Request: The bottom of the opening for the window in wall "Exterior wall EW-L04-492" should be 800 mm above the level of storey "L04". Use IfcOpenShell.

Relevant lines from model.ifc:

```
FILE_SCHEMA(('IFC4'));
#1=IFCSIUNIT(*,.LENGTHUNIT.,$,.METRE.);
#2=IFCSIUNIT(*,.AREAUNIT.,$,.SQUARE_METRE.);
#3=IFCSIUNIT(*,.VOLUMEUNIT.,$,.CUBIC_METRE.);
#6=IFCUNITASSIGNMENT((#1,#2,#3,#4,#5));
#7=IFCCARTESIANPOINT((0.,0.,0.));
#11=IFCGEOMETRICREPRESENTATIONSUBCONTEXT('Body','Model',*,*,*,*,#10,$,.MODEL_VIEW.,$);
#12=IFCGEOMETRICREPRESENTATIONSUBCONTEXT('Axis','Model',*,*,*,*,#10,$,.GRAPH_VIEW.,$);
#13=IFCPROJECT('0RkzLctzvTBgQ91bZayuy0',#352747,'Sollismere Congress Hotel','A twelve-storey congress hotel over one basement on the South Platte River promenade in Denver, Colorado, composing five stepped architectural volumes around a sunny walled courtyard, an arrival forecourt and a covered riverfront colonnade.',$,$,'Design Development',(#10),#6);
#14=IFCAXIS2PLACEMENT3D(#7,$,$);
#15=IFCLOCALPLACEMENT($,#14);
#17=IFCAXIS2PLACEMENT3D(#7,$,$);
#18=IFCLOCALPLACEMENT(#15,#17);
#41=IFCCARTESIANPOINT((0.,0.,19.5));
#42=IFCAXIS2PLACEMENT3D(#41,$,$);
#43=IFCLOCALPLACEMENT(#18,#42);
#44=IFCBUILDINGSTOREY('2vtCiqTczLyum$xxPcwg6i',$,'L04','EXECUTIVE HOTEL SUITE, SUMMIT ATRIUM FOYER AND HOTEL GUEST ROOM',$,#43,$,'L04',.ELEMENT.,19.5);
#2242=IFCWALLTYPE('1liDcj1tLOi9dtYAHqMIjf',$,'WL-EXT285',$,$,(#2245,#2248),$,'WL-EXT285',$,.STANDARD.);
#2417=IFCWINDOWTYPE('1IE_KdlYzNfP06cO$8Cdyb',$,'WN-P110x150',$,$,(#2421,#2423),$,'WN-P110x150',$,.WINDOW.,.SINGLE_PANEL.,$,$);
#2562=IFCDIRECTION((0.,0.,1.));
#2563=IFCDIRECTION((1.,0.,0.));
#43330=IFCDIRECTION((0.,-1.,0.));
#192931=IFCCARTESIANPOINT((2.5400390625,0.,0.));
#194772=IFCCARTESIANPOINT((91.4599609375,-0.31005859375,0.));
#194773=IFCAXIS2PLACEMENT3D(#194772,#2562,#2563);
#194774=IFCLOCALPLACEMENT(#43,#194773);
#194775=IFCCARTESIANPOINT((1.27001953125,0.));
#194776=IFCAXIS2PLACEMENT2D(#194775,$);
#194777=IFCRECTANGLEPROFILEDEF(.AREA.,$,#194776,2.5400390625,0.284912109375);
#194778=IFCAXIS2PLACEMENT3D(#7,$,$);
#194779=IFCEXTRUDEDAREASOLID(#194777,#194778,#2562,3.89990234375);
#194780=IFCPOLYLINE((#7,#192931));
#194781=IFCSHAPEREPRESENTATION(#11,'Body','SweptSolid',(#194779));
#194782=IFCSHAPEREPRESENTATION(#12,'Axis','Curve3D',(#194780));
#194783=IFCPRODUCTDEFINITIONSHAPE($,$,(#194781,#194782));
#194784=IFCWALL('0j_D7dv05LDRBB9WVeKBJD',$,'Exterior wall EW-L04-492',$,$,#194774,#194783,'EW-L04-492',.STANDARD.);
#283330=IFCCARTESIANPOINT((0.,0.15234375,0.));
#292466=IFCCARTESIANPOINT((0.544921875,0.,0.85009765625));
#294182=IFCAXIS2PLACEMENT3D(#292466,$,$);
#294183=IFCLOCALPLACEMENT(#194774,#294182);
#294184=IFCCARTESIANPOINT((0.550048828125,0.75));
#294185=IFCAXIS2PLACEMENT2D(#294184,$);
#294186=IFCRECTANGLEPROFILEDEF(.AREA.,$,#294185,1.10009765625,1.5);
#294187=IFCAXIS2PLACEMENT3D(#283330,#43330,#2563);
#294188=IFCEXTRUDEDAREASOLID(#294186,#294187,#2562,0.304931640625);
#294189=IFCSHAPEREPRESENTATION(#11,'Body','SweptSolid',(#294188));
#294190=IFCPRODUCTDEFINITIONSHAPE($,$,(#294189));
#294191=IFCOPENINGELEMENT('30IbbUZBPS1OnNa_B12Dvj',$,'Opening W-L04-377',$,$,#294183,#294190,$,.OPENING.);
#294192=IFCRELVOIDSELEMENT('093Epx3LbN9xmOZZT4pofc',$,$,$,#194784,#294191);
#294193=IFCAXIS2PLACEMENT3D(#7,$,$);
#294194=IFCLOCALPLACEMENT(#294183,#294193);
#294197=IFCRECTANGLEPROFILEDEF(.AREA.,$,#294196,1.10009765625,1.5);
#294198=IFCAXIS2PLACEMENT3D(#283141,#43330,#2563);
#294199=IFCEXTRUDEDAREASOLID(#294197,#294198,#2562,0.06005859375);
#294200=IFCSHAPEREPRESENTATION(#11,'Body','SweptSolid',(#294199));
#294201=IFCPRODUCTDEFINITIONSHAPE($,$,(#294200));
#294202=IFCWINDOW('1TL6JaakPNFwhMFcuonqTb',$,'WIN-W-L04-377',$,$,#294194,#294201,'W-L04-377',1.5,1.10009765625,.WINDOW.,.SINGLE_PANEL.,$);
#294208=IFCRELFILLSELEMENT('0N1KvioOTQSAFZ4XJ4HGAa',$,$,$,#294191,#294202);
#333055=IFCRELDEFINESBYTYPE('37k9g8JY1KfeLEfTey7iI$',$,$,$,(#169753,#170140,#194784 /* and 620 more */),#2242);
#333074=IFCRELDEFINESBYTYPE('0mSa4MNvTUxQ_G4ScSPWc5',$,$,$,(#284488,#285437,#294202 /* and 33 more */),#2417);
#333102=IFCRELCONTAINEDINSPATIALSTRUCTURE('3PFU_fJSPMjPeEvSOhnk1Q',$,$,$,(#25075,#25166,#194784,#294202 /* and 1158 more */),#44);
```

```python
import numpy as np
import ifcopenshell
import ifcopenshell.api.geometry
import ifcopenshell.geom
import ifcopenshell.util.element
import ifcopenshell.util.placement
import ifcopenshell.util.shape
import ifcopenshell.util.unit

model = ifcopenshell.open("model.ifc")
unit_scale = ifcopenshell.util.unit.calculate_unit_scale(model)

window = model.by_guid("1TL6JaakPNFwhMFcuonqTb")
opening = window.FillsVoids[0].RelatingOpeningElement
storey = ifcopenshell.util.element.get_container(window, ifc_class="IfcBuildingStorey")
level = ifcopenshell.util.placement.get_local_placement(storey.ObjectPlacement)[2, 3]

# The opening's origin need not be at the sill, so measure its lowest point.
shape = ifcopenshell.geom.create_shape(ifcopenshell.geom.settings(), opening)
bottom = ifcopenshell.util.shape.get_shape_bottom_elevation(shape, shape.geometry) / unit_scale
dz = level + 0.8 / unit_scale - bottom

shift = np.array([0.0, 0.0, dz])
# The window is placed relative to its opening, so it follows when the opening moves.
matrix = ifcopenshell.util.placement.get_local_placement(opening.ObjectPlacement)
matrix[:3, 3] += shift
ifcopenshell.api.geometry.edit_object_placement(
    model, product=opening, matrix=matrix, is_si=False, should_transform_children=True
)

print(f"moved by {dz * unit_scale:+.3f} m")

model.write("model_rev.ifc")
```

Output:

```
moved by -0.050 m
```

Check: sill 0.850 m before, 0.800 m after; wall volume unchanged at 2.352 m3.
